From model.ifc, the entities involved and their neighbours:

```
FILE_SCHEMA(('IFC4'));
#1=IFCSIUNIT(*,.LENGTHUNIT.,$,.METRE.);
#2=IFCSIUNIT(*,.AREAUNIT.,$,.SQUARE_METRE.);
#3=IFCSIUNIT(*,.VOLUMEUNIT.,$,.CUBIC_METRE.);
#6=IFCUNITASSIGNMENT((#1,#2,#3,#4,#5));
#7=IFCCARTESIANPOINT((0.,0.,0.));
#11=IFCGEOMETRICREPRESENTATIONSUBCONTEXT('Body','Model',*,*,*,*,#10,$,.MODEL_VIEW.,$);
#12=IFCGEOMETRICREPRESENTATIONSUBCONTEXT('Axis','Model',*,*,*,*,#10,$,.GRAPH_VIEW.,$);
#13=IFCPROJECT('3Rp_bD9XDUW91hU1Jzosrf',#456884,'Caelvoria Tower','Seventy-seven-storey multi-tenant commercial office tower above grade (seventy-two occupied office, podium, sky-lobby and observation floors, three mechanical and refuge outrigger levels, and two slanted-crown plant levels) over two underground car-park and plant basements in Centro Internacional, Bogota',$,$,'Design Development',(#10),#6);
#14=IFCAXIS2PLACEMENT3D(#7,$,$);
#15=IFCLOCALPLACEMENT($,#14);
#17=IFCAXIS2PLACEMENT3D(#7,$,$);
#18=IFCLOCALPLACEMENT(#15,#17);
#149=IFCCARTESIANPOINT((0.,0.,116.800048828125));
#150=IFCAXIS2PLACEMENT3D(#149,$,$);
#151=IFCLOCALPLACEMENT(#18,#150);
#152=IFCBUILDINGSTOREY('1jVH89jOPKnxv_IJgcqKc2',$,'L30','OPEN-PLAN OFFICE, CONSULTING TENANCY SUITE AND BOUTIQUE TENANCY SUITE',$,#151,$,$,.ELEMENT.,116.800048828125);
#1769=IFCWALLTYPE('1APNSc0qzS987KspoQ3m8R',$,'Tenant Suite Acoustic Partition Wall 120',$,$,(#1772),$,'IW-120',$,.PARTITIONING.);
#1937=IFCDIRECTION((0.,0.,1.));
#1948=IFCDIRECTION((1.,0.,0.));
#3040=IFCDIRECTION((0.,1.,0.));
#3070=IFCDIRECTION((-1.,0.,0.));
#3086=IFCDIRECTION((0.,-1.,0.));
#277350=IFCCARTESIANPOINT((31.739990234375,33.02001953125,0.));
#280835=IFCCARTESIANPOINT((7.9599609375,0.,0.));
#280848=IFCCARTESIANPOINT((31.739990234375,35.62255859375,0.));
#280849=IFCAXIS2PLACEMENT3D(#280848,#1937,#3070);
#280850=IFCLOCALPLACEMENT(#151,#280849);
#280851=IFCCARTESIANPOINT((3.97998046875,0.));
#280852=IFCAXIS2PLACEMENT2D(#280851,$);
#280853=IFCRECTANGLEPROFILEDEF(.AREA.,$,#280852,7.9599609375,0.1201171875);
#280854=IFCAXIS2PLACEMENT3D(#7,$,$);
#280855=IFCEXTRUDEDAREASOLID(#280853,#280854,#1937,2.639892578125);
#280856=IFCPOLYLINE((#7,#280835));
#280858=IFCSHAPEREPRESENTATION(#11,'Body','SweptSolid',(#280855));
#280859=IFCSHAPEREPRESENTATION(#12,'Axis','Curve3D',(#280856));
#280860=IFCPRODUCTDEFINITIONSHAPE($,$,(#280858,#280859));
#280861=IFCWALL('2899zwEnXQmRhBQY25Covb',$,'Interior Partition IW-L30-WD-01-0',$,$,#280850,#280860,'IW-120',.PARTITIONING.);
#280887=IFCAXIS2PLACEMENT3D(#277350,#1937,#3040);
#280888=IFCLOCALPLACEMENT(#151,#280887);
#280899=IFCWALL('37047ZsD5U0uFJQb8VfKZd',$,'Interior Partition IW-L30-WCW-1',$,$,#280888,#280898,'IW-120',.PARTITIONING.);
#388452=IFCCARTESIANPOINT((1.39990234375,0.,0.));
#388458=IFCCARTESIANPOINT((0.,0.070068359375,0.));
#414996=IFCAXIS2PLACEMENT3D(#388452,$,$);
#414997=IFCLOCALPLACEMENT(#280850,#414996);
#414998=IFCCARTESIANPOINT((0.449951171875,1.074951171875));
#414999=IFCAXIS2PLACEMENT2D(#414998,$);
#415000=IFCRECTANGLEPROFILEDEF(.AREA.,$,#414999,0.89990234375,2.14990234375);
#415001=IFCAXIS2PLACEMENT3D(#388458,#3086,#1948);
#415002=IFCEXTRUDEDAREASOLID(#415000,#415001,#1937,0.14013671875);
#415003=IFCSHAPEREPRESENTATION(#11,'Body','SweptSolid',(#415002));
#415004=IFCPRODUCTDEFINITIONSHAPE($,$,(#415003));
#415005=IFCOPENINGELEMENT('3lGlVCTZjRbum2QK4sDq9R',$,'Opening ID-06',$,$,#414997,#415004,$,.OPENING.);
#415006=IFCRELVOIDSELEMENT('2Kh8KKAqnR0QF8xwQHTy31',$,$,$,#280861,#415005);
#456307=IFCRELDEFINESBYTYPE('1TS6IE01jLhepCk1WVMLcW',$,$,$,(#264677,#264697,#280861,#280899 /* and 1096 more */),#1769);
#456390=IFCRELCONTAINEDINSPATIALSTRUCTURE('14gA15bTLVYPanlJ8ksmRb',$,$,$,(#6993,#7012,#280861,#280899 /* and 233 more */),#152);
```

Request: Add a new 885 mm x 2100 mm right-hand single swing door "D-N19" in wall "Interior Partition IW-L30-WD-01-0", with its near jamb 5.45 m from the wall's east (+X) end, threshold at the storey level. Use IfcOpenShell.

```python
import numpy as np
import ifcopenshell
import ifcopenshell.api.feature
import ifcopenshell.api.geometry
import ifcopenshell.api.root
import ifcopenshell.api.spatial
import ifcopenshell.geom
import ifcopenshell.util.element
import ifcopenshell.util.placement
import ifcopenshell.util.representation
import ifcopenshell.util.shape
import ifcopenshell.util.unit

model = ifcopenshell.open("model.ifc")
unit_scale = ifcopenshell.util.unit.calculate_unit_scale(model)
settings = ifcopenshell.geom.settings()


def volume(element):
    """Net volume in cubic metres, openings subtracted."""
    shape = ifcopenshell.geom.create_shape(settings, element)
    return ifcopenshell.util.shape.get_volume(shape.geometry)


wall = model.by_id(280861)
storey = ifcopenshell.util.element.get_container(wall, ifc_class="IfcBuildingStorey")
context = ifcopenshell.util.representation.get_context(model, "Model", "Body", "MODEL_VIEW")
before = volume(wall)

width, height, from_end, sill = 0.885, 2.1, 5.45, 0.0  # metres

# The wall runs along its own X axis, and the end named is its -X end.
wall_shape = ifcopenshell.geom.create_shape(settings, wall)
x, y, z = ifcopenshell.util.shape.get_vertices(wall_shape.geometry).T
start = x.min() + from_end
face, thickness = float(y.min()), float(y.max() - y.min())
wall_matrix = ifcopenshell.util.placement.get_local_placement(wall.ObjectPlacement)
level = ifcopenshell.util.placement.get_local_placement(storey.ObjectPlacement)[2, 3]


def in_wall(x, y):
    """Placement at x, y metres in the wall's axes, at sill height."""
    matrix = wall_matrix.copy()
    matrix[:, 3] = wall_matrix @ np.array([x / unit_scale, y / unit_scale, 0.0, 1.0])
    matrix[2, 3] = level + sill / unit_scale
    return matrix


# Opening: a box that overshoots both wall faces by 50 mm.
opening = ifcopenshell.api.root.create_entity(model, ifc_class="IfcOpeningElement", predefined_type="OPENING")
box = ifcopenshell.api.geometry.add_wall_representation(
    model, context=context, length=width, height=height, thickness=thickness + 0.1
)
ifcopenshell.api.geometry.assign_representation(model, product=opening, representation=box)
ifcopenshell.api.geometry.edit_object_placement(model, product=opening, matrix=in_wall(start, face - 0.05), is_si=False)
ifcopenshell.api.feature.add_feature(model, feature=opening, element=wall)

door = ifcopenshell.api.root.create_entity(model, ifc_class="IfcDoor", name="D-N19", predefined_type="DOOR")
door.OverallWidth, door.OverallHeight = width / unit_scale, height / unit_scale
door.OperationType = "SINGLE_SWING_RIGHT"
body = ifcopenshell.api.geometry.add_door_representation(
    model,
    context=context,
    overall_width=door.OverallWidth,
    overall_height=door.OverallHeight,
    operation_type="SINGLE_SWING_RIGHT",
    lining_properties={"LiningDepth": thickness / unit_scale, "ThresholdDepth": thickness / unit_scale},
)
ifcopenshell.api.geometry.assign_representation(model, product=door, representation=body)
ifcopenshell.api.spatial.assign_container(model, products=[door], relating_structure=storey)
ifcopenshell.api.feature.add_filling(model, opening=opening, element=door)

# The lining spans the wall, so the door starts at the wall face.
ifcopenshell.api.geometry.edit_object_placement(model, product=door, matrix=in_wall(start, face), is_si=False)

after = volume(wall)

print(f"wall volume {before:.3f} -> {after:.3f} m3")

model.write("model_rev.ifc")
```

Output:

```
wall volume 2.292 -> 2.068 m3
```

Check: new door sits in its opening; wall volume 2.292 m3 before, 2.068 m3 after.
